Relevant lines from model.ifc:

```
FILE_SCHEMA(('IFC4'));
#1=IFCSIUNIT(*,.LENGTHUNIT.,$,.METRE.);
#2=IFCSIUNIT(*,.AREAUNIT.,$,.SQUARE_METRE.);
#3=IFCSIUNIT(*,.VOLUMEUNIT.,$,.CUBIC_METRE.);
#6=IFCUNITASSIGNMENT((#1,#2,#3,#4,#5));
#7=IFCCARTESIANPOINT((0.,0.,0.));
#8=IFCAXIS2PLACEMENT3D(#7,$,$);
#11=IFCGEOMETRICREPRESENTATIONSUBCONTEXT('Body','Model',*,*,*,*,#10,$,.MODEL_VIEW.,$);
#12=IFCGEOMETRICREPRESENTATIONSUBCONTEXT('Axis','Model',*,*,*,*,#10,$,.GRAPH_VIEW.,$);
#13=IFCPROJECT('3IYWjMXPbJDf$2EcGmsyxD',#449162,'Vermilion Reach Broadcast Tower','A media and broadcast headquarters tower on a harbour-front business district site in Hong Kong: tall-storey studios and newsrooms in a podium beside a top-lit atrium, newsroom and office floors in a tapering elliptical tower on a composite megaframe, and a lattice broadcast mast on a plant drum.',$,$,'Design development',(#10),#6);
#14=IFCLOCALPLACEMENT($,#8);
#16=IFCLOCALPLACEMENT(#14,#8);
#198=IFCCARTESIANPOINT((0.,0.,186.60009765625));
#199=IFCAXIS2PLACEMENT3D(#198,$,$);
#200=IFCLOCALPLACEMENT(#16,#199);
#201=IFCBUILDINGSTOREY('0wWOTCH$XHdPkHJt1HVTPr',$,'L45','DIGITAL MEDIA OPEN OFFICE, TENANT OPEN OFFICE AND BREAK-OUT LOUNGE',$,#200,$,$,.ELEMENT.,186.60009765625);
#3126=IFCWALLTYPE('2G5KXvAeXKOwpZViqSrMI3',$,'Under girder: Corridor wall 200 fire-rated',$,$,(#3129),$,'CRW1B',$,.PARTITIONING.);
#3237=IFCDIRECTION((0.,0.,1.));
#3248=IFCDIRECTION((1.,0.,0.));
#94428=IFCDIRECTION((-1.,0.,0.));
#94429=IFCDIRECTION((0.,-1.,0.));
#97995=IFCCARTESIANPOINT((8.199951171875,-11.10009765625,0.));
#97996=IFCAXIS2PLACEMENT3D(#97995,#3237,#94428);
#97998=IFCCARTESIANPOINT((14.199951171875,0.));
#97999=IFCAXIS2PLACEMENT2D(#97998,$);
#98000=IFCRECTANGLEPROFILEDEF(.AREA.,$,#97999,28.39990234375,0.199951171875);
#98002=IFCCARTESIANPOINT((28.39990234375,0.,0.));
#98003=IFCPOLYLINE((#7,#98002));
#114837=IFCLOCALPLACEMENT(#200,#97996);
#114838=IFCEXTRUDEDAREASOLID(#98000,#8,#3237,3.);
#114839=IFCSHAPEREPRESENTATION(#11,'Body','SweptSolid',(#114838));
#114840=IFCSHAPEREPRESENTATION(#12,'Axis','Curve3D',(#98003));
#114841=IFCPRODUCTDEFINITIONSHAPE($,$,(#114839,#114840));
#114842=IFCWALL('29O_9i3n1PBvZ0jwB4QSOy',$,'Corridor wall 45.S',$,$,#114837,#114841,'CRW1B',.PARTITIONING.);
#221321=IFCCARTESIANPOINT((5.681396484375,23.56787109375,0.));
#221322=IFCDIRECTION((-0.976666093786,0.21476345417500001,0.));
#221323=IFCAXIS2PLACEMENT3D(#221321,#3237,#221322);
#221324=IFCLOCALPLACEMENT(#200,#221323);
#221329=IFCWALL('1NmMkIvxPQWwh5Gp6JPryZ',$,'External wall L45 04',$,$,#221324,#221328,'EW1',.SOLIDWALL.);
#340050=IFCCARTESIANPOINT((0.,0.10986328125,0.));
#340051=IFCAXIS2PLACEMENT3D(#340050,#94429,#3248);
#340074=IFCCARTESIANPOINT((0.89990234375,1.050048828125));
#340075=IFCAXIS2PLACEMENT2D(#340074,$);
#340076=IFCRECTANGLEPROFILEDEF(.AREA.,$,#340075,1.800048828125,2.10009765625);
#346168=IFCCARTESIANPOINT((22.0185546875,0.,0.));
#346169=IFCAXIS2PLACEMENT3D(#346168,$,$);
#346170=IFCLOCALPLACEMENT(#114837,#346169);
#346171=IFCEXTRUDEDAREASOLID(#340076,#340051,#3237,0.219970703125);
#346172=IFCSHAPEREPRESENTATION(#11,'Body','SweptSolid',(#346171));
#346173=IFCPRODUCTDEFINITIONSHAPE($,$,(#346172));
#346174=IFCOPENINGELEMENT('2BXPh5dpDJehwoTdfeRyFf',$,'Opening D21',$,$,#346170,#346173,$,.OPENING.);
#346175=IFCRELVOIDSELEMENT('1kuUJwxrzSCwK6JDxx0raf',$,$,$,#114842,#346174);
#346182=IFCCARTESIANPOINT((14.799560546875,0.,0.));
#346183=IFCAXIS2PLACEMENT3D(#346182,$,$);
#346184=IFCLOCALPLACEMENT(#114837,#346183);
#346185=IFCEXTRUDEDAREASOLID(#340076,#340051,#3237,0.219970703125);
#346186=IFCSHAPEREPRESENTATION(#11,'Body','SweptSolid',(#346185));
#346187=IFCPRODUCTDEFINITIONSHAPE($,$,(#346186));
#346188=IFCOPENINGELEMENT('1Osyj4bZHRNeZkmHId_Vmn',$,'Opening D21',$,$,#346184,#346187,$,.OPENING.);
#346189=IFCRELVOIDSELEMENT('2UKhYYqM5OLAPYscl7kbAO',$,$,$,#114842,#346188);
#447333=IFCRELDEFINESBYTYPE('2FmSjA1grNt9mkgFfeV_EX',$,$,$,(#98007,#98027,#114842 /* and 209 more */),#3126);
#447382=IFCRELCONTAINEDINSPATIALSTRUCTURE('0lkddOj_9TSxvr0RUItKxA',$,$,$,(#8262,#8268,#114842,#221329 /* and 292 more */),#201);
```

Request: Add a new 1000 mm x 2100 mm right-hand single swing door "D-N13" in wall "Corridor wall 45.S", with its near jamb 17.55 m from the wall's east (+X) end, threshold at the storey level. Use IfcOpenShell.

```python
import numpy as np
import ifcopenshell
import ifcopenshell.api.feature
import ifcopenshell.api.geometry
import ifcopenshell.api.root
import ifcopenshell.api.spatial
import ifcopenshell.geom
import ifcopenshell.util.element
import ifcopenshell.util.placement
import ifcopenshell.util.representation
import ifcopenshell.util.shape
import ifcopenshell.util.unit

model = ifcopenshell.open("model.ifc")
unit_scale = ifcopenshell.util.unit.calculate_unit_scale(model)
settings = ifcopenshell.geom.settings()


def volume(element):
    """Net volume in cubic metres, openings subtracted."""
    shape = ifcopenshell.geom.create_shape(settings, element)
    return ifcopenshell.util.shape.get_volume(shape.geometry)


wall = model.by_guid("29O_9i3n1PBvZ0jwB4QSOy")
storey = ifcopenshell.util.element.get_container(wall, ifc_class="IfcBuildingStorey")
context = ifcopenshell.util.representation.get_context(model, "Model", "Body", "MODEL_VIEW")
before = volume(wall)

width, height, from_end, sill = 1, 2.1, 17.55, 0.0  # metres

# The wall runs along its own X axis, and the end named is its -X end.
wall_shape = ifcopenshell.geom.create_shape(settings, wall)
x, y, z = ifcopenshell.util.shape.get_vertices(wall_shape.geometry).T
start = x.min() + from_end
face, thickness = float(y.min()), float(y.max() - y.min())
wall_matrix = ifcopenshell.util.placement.get_local_placement(wall.ObjectPlacement)
level = ifcopenshell.util.placement.get_local_placement(storey.ObjectPlacement)[2, 3]


def in_wall(x, y):
    """Placement at x, y metres in the wall's axes, at sill height."""
    matrix = wall_matrix.copy()
    matrix[:, 3] = wall_matrix @ np.array([x / unit_scale, y / unit_scale, 0.0, 1.0])
    matrix[2, 3] = level + sill / unit_scale
    return matrix


# Opening: a box that overshoots both wall faces by 50 mm.
opening = ifcopenshell.api.root.create_entity(model, ifc_class="IfcOpeningElement", predefined_type="OPENING")
box = ifcopenshell.api.geometry.add_wall_representation(
    model, context=context, length=width, height=height, thickness=thickness + 0.1
)
ifcopenshell.api.geometry.assign_representation(model, product=opening, representation=box)
ifcopenshell.api.geometry.edit_object_placement(model, product=opening, matrix=in_wall(start, face - 0.05), is_si=False)
ifcopenshell.api.feature.add_feature(model, feature=opening, element=wall)

door = ifcopenshell.api.root.create_entity(model, ifc_class="IfcDoor", name="D-N13", predefined_type="DOOR")
door.OverallWidth, door.OverallHeight = width / unit_scale, height / unit_scale
door.OperationType = "SINGLE_SWING_RIGHT"
body = ifcopenshell.api.geometry.add_door_representation(
    model,
    context=context,
    overall_width=door.OverallWidth,
    overall_height=door.OverallHeight,
    operation_type="SINGLE_SWING_RIGHT",
    lining_properties={"LiningDepth": thickness / unit_scale, "ThresholdDepth": thickness / unit_scale},
)
ifcopenshell.api.geometry.assign_representation(model, product=door, representation=body)
ifcopenshell.api.spatial.assign_container(model, products=[door], relating_structure=storey)
ifcopenshell.api.feature.add_filling(model, opening=opening, element=door)

# The lining spans the wall, so the door starts at the wall face.
ifcopenshell.api.geometry.edit_object_placement(model, product=door, matrix=in_wall(start, face), is_si=False)

after = volume(wall)

print(f"wall volume {before:.3f} -> {after:.3f} m3")

model.write("model_edited.ifc")
```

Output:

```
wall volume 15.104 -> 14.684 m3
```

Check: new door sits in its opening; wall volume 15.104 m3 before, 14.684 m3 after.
